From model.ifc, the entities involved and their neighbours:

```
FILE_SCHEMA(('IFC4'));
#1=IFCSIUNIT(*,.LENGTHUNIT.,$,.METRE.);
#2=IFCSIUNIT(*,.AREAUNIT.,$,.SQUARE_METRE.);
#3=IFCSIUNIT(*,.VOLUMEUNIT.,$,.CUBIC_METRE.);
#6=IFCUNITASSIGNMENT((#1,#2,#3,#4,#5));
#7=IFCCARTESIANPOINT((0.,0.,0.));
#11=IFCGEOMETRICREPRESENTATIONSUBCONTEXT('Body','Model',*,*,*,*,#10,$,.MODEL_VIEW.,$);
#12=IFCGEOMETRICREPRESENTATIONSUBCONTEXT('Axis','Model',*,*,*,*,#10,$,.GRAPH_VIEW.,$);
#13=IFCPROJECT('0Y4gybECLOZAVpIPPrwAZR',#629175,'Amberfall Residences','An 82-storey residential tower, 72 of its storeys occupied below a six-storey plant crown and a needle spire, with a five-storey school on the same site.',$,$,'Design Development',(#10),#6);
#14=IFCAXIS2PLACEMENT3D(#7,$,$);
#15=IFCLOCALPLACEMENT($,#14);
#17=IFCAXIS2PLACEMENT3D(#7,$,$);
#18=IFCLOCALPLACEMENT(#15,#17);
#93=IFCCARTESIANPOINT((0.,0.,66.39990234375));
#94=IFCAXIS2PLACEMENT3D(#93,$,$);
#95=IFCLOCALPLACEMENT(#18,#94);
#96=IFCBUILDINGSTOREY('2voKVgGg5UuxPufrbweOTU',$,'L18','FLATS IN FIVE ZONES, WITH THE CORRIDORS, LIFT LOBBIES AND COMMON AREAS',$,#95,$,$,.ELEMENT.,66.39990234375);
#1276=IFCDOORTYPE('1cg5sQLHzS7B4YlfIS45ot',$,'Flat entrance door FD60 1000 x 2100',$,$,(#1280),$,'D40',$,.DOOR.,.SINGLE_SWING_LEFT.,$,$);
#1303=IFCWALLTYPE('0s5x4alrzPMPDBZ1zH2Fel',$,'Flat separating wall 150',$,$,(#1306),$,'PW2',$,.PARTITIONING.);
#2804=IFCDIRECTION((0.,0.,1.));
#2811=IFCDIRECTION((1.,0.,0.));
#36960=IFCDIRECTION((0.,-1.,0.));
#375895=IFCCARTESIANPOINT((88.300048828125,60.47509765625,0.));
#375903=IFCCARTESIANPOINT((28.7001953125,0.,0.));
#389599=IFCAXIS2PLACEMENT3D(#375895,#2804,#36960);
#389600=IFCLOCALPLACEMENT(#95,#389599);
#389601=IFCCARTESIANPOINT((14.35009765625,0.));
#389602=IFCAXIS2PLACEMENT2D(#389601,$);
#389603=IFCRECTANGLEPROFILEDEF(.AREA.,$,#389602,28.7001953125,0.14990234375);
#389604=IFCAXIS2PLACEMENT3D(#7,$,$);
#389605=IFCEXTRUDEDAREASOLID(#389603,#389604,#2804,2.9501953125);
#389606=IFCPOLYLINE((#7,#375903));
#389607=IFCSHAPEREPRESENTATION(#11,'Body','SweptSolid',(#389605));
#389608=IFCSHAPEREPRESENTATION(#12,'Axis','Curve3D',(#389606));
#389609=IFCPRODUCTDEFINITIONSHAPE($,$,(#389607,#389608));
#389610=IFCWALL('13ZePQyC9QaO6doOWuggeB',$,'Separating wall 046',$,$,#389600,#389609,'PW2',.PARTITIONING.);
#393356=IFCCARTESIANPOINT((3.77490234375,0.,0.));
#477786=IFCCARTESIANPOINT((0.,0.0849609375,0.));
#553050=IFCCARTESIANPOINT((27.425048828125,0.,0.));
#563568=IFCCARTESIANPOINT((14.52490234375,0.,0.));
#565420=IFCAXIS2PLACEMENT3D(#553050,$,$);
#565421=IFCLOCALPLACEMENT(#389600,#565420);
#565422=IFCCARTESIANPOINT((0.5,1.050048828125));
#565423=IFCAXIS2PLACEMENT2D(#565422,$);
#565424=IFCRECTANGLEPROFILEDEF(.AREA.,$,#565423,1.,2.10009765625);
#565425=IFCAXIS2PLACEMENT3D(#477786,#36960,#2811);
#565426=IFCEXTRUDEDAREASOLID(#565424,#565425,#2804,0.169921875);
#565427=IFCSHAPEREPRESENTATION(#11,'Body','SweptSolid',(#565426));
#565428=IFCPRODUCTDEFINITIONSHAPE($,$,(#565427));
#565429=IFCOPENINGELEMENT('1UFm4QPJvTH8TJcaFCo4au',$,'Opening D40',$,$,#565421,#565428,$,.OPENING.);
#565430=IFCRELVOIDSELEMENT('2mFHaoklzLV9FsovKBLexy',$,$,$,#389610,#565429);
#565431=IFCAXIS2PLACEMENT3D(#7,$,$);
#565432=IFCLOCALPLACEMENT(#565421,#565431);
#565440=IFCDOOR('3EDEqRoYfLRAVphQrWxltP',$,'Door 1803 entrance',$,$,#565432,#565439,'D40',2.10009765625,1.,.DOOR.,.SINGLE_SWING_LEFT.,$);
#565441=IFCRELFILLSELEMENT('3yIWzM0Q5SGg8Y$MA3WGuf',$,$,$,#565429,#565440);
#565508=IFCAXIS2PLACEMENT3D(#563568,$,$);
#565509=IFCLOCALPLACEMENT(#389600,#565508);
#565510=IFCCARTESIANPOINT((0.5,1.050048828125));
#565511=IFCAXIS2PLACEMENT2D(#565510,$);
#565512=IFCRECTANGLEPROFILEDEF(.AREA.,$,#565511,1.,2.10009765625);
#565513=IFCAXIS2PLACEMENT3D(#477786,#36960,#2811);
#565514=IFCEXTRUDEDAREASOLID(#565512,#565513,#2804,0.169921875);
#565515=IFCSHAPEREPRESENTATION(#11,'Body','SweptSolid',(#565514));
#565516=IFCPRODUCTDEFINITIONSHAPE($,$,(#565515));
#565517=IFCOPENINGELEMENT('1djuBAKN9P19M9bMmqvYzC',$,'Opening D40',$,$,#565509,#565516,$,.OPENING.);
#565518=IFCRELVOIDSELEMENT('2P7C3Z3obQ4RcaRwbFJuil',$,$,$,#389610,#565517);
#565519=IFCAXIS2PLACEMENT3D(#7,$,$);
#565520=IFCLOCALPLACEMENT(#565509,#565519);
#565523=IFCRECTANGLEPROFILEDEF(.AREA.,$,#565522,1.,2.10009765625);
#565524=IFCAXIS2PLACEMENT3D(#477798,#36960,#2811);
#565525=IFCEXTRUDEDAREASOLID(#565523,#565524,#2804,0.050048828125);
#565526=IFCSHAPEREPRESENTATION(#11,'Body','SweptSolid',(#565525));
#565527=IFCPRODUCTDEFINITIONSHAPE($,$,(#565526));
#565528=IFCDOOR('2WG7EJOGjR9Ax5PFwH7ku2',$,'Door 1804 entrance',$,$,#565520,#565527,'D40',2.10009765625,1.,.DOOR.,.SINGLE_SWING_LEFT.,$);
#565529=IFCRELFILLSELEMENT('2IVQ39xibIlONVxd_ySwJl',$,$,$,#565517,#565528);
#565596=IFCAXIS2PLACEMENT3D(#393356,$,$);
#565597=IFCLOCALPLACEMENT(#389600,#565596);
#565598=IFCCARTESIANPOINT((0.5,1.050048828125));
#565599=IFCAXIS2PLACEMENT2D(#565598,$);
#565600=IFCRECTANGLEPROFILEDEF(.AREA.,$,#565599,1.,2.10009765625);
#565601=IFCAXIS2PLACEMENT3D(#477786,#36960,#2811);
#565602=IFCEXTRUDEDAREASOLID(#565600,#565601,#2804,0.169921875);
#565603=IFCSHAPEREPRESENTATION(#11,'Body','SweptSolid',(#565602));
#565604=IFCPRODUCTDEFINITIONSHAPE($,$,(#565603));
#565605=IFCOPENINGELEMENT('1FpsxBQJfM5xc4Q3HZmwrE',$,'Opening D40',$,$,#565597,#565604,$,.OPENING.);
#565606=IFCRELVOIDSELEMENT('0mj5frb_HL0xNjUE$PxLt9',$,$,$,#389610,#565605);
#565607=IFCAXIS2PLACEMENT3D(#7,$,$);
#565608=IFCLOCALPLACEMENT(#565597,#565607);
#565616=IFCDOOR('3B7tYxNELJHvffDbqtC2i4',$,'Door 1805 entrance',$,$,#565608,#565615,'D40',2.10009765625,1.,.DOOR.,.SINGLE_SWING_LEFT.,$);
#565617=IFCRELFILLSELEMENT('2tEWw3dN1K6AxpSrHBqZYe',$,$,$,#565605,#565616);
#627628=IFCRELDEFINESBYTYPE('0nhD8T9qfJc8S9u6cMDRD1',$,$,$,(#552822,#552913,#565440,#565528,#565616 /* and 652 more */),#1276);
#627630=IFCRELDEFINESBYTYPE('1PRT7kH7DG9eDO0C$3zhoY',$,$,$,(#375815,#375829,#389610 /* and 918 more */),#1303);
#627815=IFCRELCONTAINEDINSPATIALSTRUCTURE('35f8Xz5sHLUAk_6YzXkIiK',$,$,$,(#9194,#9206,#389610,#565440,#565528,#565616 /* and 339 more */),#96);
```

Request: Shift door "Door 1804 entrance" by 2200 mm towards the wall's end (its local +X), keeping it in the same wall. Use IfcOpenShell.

```python
import ifcopenshell
import ifcopenshell.api.geometry
import ifcopenshell.util.placement
import ifcopenshell.util.unit

model = ifcopenshell.open("model.ifc")
unit_scale = ifcopenshell.util.unit.calculate_unit_scale(model)

door = model.by_id(565528)
opening = door.FillsVoids[0].RelatingOpeningElement
wall = opening.VoidsElements[0].RelatingBuildingElement

wall_matrix = ifcopenshell.util.placement.get_local_placement(wall.ObjectPlacement)
shift = wall_matrix[:3, 0] * 2.2 / unit_scale
before = ifcopenshell.util.placement.get_local_placement(door.ObjectPlacement)[:3, 3].copy()

# The door is placed relative to its opening, so it follows when the opening moves.
matrix = ifcopenshell.util.placement.get_local_placement(opening.ObjectPlacement)
matrix[:3, 3] += shift
ifcopenshell.api.geometry.edit_object_placement(
    model, product=opening, matrix=matrix, is_si=False, should_transform_children=True
)

after = ifcopenshell.util.placement.get_local_placement(door.ObjectPlacement)[:3, 3]
print("door moved by", (after - before).round(3) + 0.0)

model.write("model_updated.ifc")
```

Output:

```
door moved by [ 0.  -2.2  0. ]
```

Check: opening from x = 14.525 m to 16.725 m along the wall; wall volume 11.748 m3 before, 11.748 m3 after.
